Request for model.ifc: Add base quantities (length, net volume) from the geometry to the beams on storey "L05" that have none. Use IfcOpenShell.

First a look at what the model holds.

```python
import ifcopenshell
import ifcopenshell.util.element
import ifcopenshell.util.unit

model = ifcopenshell.open("model.ifc")
print(model.schema)
for unit_type in ("LENGTHUNIT", "AREAUNIT", "VOLUMEUNIT"):
    print(unit_type, ifcopenshell.util.unit.calculate_unit_scale(model, unit_type))
storey = next(s for s in model.by_type("IfcBuildingStorey") if s.Name == "L05")
beams = [e for e in ifcopenshell.util.element.get_decomposition(storey) if e.is_a("IfcBeam")]
for e in sorted(beams, key=lambda e: e.id()):
    print(e.id(), e.is_a(), e.Name, list(ifcopenshell.util.element.get_psets(e, qtos_only=True)), sep=" | ")
```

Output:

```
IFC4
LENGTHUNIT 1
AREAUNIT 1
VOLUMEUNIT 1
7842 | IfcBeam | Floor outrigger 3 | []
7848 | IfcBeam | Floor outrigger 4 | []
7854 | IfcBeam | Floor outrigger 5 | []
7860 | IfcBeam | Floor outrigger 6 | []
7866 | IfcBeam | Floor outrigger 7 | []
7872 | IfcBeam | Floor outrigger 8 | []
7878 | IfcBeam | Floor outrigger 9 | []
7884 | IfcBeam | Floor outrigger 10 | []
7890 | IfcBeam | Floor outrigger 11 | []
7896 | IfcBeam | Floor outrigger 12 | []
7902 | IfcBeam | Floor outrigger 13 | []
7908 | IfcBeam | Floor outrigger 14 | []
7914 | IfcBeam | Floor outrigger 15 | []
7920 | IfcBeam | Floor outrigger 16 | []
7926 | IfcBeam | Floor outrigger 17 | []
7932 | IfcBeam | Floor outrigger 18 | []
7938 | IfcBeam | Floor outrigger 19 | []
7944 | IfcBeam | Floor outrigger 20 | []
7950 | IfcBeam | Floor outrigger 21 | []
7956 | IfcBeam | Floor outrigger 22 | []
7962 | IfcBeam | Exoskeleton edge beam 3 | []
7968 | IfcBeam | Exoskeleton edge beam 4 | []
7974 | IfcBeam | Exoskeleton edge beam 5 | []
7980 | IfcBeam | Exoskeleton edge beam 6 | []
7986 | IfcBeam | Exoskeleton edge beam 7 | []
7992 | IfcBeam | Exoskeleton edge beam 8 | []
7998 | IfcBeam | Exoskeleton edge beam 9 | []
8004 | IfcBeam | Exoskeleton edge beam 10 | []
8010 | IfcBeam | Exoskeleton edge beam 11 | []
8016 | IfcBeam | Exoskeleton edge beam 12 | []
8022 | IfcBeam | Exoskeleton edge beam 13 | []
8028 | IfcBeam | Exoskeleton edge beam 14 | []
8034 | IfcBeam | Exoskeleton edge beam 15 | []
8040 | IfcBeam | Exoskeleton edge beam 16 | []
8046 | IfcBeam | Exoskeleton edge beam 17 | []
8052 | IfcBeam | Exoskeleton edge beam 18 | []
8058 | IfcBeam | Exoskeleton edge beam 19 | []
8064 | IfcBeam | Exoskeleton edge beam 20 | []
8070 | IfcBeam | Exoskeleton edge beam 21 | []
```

```python
import ifcopenshell
import ifcopenshell.api.pset
import ifcopenshell.geom
import ifcopenshell.util.element
import ifcopenshell.util.shape
import ifcopenshell.util.unit

model = ifcopenshell.open("model.ifc")
unit_scale = ifcopenshell.util.unit.calculate_unit_scale(model)
volume_scale = ifcopenshell.util.unit.calculate_unit_scale(model, "VOLUMEUNIT")
settings = ifcopenshell.geom.settings()

storey = next(s for s in model.by_type("IfcBuildingStorey") if s.Name == "L05")
beams = [e for e in ifcopenshell.util.element.get_decomposition(storey) if e.is_a("IfcBeam")]

for e in sorted(beams, key=lambda e: e.id()):
    if ifcopenshell.util.element.get_psets(e, qtos_only=True, should_inherit=False):
        continue
    # Geometry comes back in metres, in the element's own axes.
    shape = ifcopenshell.geom.create_shape(settings, e)
    values = {
        "Length": ifcopenshell.util.shape.get_max_xyz(shape.geometry) / unit_scale,
        "NetVolume": ifcopenshell.util.shape.get_volume(shape.geometry) / volume_scale,
    }
    qto = ifcopenshell.api.pset.add_qto(model, product=e, name="Qto_BeamBaseQuantities")
    ifcopenshell.api.pset.edit_qto(model, qto=qto, properties=values)
    print(e.id(), {k: round(v, 3) for k, v in values.items()})

model.write("model-out.ifc")
```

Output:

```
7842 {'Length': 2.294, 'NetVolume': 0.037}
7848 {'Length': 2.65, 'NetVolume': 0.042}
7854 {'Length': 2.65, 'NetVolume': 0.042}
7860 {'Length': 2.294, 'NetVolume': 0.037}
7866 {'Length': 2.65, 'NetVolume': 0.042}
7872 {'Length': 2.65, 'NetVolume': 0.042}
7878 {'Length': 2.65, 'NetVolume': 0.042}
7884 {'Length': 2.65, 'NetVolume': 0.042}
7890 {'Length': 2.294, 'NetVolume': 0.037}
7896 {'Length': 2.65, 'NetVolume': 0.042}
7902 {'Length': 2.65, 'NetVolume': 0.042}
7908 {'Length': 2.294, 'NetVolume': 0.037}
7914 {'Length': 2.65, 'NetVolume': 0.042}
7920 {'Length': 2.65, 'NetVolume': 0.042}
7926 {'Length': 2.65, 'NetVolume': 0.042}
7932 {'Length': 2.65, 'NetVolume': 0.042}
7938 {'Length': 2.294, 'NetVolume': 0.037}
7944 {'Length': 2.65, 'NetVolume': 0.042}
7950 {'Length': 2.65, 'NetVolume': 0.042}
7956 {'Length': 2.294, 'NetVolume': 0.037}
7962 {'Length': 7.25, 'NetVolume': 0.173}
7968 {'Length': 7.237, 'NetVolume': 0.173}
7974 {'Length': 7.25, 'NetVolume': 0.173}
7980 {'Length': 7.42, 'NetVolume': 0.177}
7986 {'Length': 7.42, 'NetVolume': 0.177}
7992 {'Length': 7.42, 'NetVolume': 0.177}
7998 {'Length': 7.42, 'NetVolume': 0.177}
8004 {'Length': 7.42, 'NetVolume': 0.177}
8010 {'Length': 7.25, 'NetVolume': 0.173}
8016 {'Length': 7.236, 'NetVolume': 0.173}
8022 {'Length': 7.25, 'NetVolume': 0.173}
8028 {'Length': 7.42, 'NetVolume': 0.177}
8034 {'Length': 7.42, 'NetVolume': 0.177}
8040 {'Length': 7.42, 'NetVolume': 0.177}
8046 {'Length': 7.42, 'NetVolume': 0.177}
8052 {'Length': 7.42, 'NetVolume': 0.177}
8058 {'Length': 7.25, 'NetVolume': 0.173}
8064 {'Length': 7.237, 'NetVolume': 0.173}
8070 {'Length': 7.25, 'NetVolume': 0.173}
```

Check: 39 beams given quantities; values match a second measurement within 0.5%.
